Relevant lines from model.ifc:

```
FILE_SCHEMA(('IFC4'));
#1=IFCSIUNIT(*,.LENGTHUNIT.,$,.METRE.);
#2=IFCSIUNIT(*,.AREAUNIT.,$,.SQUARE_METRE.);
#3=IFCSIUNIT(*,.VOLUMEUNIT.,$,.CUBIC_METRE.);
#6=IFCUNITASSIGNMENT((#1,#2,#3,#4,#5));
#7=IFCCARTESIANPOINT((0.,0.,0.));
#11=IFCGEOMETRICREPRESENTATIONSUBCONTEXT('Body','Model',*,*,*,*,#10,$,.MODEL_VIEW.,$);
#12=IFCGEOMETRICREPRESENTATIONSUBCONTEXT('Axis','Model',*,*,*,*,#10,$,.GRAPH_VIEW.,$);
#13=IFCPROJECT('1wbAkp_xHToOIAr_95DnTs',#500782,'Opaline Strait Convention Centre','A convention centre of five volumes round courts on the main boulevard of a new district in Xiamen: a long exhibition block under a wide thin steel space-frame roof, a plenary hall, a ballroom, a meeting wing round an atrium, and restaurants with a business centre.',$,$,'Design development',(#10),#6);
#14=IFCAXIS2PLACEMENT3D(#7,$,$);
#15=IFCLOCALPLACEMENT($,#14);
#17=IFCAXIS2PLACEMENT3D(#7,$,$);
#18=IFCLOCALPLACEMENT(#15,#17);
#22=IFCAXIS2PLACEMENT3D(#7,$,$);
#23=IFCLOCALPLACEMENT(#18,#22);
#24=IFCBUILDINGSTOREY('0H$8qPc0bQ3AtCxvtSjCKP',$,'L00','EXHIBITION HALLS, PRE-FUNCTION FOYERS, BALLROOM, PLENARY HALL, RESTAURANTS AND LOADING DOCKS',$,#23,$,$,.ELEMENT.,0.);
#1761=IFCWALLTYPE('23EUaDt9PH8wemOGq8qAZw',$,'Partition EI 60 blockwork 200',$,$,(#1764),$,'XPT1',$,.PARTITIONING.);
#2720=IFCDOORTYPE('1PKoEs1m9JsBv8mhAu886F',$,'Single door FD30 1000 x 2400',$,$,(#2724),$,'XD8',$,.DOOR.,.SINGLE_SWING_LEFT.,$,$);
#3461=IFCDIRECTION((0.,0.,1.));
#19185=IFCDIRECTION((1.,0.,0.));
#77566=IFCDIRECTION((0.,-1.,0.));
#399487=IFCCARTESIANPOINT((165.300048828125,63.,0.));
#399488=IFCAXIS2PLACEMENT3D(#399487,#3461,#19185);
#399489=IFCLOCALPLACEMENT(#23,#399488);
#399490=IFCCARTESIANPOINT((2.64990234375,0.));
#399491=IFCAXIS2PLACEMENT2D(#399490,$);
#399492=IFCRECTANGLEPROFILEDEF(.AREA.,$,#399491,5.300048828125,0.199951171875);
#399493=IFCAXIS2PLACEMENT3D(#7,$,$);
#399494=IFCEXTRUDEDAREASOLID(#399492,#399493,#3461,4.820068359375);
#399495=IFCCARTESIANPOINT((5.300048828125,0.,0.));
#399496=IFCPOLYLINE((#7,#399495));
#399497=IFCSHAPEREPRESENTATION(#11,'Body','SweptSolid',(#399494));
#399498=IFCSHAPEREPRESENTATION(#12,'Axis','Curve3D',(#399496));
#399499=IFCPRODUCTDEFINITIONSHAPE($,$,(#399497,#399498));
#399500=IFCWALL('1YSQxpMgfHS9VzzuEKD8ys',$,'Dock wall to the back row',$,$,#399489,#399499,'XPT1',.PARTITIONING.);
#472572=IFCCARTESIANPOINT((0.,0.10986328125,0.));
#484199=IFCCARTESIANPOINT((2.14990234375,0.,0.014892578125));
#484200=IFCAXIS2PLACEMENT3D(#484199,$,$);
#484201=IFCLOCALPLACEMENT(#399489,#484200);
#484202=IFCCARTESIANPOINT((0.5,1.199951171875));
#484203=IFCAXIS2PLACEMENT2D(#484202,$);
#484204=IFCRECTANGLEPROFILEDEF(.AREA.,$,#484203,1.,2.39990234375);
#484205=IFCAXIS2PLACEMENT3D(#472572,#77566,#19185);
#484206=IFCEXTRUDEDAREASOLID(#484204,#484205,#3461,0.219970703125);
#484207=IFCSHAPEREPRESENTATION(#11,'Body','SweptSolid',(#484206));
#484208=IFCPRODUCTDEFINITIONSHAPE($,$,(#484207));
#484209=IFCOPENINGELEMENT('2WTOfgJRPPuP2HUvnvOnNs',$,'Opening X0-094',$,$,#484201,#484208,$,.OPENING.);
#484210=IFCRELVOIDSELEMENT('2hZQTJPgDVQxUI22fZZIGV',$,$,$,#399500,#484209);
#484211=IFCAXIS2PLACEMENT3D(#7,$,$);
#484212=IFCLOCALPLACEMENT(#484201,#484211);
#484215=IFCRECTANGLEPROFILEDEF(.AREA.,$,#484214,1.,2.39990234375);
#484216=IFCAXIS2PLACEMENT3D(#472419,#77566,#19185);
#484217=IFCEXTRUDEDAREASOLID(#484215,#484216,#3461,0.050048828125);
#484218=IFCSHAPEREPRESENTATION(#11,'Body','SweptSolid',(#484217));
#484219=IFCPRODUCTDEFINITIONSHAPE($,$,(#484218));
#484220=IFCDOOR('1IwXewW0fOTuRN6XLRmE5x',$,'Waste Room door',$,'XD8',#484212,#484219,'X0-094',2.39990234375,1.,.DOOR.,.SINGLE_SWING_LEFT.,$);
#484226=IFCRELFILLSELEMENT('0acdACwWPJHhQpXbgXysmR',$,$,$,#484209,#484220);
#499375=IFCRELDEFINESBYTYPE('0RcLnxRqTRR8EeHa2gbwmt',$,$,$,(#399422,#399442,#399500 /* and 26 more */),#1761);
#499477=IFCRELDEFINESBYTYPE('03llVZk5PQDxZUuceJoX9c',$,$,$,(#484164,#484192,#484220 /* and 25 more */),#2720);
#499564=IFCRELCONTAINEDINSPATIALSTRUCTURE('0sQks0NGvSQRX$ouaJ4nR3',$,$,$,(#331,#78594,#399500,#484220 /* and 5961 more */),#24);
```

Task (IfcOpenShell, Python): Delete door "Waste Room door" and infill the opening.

```python
import ifcopenshell
import ifcopenshell.api.feature
import ifcopenshell.api.root
import ifcopenshell.geom
import ifcopenshell.util.shape

model = ifcopenshell.open("model.ifc")
settings = ifcopenshell.geom.settings()


def volume(element):
    """Net volume in cubic metres, openings subtracted."""
    shape = ifcopenshell.geom.create_shape(settings, element)
    return ifcopenshell.util.shape.get_volume(shape.geometry)


door = model.by_guid("1IwXewW0fOTuRN6XLRmE5x")
opening = door.FillsVoids[0].RelatingOpeningElement
wall = opening.VoidsElements[0].RelatingBuildingElement
before = volume(wall)

ifcopenshell.api.root.remove_product(model, product=door)
ifcopenshell.api.feature.remove_feature(model, feature=opening)

after = volume(wall)

print(f"wall volume {before:.3f} -> {after:.3f} m3")

model.write("model-out.ifc")
```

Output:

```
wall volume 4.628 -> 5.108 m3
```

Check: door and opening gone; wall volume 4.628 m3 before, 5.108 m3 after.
